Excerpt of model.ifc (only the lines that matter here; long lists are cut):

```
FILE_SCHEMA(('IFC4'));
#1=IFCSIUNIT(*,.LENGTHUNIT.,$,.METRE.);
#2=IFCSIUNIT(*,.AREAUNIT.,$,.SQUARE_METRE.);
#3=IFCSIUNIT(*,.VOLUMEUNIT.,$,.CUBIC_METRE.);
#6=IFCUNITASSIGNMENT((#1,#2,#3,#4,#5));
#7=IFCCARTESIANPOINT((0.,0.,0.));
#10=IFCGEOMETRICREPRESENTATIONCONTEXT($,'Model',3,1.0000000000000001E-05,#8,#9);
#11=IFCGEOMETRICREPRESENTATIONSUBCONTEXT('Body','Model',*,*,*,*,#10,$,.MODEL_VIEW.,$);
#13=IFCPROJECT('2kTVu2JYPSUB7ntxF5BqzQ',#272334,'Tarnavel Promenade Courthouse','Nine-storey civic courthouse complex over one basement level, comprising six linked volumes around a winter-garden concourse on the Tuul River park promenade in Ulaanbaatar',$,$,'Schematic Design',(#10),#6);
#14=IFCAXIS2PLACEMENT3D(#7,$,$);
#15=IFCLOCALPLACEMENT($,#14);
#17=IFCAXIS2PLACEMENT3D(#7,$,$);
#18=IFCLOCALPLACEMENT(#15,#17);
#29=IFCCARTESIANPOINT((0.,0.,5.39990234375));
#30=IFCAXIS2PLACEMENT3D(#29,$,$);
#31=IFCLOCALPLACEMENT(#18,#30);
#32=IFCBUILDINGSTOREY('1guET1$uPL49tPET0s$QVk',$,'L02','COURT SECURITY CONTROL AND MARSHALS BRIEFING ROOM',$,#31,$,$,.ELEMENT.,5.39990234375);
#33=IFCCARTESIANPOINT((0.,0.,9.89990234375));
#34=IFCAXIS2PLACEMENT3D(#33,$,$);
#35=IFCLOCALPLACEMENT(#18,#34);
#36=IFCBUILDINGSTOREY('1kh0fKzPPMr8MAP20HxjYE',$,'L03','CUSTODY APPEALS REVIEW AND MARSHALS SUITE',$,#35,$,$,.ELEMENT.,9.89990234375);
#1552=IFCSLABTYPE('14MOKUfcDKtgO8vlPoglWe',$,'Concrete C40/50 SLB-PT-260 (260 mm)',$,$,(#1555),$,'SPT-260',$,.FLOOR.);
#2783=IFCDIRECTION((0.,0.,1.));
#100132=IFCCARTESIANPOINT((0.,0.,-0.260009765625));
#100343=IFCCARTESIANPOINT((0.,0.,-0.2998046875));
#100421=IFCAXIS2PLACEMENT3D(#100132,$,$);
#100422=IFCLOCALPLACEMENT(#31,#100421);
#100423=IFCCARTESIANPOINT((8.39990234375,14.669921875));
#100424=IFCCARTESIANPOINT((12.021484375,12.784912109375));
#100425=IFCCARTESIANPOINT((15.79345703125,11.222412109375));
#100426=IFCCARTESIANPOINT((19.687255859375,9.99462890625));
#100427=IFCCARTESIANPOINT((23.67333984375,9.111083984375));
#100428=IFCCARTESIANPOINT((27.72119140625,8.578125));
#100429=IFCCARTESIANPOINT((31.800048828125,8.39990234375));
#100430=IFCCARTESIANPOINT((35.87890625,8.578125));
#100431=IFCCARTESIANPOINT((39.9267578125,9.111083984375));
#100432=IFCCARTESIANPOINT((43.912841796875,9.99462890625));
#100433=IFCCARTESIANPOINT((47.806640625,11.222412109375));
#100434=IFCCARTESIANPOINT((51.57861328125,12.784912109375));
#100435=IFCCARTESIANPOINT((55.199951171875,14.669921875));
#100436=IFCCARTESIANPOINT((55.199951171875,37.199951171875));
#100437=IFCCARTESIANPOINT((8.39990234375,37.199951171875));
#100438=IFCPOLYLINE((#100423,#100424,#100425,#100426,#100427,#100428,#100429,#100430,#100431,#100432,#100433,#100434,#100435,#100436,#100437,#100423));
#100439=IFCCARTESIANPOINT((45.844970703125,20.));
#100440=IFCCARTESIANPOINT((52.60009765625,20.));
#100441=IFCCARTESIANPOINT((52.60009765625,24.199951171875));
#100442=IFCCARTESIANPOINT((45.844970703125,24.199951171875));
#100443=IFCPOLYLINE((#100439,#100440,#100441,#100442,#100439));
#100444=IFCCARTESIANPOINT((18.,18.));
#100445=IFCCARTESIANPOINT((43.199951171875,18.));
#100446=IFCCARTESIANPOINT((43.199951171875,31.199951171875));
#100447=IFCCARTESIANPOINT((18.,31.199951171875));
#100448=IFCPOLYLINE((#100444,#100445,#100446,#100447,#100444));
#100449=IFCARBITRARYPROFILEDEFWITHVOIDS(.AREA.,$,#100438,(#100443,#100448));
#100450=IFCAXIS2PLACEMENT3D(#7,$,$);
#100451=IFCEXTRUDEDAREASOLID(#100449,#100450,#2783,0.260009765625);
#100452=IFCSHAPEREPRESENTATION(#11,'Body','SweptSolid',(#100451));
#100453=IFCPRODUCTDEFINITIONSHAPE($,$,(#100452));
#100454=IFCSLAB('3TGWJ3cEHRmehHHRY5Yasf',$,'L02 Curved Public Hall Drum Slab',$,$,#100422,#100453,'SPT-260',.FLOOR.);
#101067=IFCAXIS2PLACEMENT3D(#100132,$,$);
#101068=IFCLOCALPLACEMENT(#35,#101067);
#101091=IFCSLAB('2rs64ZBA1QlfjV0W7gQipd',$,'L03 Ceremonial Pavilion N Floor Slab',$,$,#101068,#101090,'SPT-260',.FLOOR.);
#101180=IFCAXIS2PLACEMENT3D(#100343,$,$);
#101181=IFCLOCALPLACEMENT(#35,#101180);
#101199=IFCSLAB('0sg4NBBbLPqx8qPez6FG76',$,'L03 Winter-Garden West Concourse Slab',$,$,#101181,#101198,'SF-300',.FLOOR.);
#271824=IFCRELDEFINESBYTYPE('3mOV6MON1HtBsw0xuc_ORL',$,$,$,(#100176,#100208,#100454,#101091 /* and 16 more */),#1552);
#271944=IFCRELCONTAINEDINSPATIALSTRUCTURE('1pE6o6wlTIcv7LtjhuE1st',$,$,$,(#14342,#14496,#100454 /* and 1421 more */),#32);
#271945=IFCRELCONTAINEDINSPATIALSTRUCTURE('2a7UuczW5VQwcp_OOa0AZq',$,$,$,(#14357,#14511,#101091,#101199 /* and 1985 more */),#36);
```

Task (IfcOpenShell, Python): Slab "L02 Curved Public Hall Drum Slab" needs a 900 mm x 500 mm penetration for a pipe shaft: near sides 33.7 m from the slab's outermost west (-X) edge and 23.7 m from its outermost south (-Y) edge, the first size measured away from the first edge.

```python
import numpy as np
import ifcopenshell
import ifcopenshell.api.feature
import ifcopenshell.api.geometry
import ifcopenshell.api.root
import ifcopenshell.geom
import ifcopenshell.util.placement
import ifcopenshell.util.representation
import ifcopenshell.util.shape
import ifcopenshell.util.unit

model = ifcopenshell.open("model.ifc")
unit_scale = ifcopenshell.util.unit.calculate_unit_scale(model)
settings = ifcopenshell.geom.settings()


def volume(element):
    """Net volume in cubic metres, openings subtracted."""
    shape = ifcopenshell.geom.create_shape(settings, element)
    return ifcopenshell.util.shape.get_volume(shape.geometry)


slab = model.by_guid("3TGWJ3cEHRmehHHRY5Yasf")
before = volume(slab)

# Extent in the slab's own axes, in metres. The edges named are its -X and -Y sides.
slab_shape = ifcopenshell.geom.create_shape(settings, slab)
vertices = ifcopenshell.util.shape.get_vertices(slab_shape.geometry)
x_min, y_min, bottom = vertices.min(axis=0)
top = vertices[:, 2].max()

opening = ifcopenshell.api.root.create_entity(model, ifc_class="IfcOpeningElement", name="Pipe shaft opening", predefined_type="OPENING")
context = ifcopenshell.util.representation.get_context(model, "Model", "Body", "MODEL_VIEW")
width, depth = 0.9, 0.5
outline = [(0.0, 0.0), (width, 0.0), (width, depth), (0.0, depth), (0.0, 0.0)]
# Overshoot both faces by 50 mm so the cut is clean.
shape = ifcopenshell.api.geometry.add_slab_representation(
    model, context=context, depth=top - bottom + 0.1, polyline=outline
)
ifcopenshell.api.geometry.assign_representation(model, product=opening, representation=shape)

matrix = ifcopenshell.util.placement.get_local_placement(slab.ObjectPlacement)
matrix[:, 3] = matrix @ np.append(np.array([x_min + 33.7, y_min + 23.7, bottom - 0.05]) / unit_scale, 1.0)
ifcopenshell.api.geometry.edit_object_placement(model, product=opening, matrix=matrix, is_si=False)
ifcopenshell.api.feature.add_feature(model, feature=opening, element=slab)

after = volume(slab)

print(f"slab volume {before:.3f} -> {after:.3f} m3")

model.write("model_v2.ifc")
```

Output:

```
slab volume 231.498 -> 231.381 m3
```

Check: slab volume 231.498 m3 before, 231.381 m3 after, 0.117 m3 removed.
